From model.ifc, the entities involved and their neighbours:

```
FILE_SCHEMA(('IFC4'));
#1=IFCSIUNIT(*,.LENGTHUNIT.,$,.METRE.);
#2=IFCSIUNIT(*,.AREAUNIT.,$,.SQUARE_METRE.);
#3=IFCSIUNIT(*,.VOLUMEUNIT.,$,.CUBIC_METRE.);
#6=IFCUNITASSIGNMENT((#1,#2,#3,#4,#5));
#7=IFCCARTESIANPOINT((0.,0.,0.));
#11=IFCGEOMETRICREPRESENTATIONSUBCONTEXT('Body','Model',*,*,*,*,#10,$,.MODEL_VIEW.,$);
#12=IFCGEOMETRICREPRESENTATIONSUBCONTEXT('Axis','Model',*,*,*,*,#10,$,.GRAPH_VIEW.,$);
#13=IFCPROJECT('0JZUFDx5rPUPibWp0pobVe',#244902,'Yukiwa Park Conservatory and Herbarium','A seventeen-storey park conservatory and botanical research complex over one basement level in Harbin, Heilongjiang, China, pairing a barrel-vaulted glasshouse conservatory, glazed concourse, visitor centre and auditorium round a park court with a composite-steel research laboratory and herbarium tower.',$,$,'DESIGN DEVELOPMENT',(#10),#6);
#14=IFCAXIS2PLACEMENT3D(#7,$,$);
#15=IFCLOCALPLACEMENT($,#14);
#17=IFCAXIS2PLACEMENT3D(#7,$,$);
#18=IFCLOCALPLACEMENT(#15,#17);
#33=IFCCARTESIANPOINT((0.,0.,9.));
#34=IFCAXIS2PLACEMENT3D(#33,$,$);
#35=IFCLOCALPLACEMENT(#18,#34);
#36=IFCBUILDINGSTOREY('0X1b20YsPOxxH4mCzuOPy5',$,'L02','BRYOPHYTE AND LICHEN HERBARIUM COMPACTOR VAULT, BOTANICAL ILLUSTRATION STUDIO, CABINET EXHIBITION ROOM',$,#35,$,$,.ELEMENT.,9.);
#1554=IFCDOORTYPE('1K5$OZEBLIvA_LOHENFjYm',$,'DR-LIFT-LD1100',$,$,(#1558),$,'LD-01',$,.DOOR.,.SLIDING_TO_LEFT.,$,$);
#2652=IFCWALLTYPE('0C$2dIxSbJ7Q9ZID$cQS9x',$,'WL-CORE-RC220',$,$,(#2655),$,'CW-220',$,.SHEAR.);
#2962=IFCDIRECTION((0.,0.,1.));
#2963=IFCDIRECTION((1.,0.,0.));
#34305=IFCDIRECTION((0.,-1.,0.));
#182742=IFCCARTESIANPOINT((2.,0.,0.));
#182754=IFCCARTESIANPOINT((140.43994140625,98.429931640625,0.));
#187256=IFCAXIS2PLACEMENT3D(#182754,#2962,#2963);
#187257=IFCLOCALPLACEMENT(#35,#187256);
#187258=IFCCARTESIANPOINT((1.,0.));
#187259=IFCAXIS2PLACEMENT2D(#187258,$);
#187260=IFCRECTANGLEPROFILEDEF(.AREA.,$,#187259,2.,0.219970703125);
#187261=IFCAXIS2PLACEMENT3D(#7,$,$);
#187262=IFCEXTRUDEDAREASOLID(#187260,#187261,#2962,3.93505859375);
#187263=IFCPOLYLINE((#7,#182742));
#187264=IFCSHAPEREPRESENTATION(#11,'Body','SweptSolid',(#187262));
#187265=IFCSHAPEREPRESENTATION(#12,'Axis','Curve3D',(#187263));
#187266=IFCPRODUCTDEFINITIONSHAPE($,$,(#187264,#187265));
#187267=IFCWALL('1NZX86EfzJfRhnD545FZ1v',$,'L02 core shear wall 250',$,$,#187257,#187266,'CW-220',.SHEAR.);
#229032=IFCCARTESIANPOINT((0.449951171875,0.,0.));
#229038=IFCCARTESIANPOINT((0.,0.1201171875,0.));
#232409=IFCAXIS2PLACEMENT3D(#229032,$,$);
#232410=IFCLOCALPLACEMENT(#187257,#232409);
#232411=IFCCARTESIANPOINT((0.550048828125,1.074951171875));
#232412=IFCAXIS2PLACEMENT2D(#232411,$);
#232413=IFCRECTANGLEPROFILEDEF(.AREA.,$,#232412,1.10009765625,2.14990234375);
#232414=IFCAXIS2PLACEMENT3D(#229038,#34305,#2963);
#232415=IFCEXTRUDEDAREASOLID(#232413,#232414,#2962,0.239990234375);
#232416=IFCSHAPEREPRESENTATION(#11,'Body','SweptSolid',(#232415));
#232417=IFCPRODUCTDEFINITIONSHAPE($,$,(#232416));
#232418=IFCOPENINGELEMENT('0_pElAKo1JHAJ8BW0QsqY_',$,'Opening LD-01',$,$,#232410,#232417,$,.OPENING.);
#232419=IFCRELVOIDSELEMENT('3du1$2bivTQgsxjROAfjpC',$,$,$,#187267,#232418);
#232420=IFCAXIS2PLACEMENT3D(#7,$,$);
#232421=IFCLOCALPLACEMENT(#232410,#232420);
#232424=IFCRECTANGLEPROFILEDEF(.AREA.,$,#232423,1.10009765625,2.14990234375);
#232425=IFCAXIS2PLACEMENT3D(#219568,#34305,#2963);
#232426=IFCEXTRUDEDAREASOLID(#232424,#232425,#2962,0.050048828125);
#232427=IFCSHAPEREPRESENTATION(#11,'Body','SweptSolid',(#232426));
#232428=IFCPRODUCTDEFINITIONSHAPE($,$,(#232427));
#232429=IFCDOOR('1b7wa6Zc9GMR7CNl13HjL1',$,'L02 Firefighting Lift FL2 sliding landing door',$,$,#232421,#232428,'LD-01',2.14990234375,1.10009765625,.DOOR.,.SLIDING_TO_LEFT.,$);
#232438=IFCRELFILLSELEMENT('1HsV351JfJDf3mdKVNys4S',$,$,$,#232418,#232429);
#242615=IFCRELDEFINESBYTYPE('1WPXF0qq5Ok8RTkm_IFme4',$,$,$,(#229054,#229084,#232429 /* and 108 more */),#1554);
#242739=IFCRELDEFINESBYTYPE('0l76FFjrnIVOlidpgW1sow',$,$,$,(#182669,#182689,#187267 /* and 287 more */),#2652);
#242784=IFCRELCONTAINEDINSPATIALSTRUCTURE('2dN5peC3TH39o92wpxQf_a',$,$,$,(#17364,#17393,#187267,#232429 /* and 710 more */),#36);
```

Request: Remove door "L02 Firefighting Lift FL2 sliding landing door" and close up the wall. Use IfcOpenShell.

```python
import ifcopenshell
import ifcopenshell.api.feature
import ifcopenshell.api.root
import ifcopenshell.geom
import ifcopenshell.util.shape

model = ifcopenshell.open("model.ifc")
settings = ifcopenshell.geom.settings()


def volume(element):
    """Net volume in cubic metres, openings subtracted."""
    shape = ifcopenshell.geom.create_shape(settings, element)
    return ifcopenshell.util.shape.get_volume(shape.geometry)


door = model.by_id(232429)
opening = door.FillsVoids[0].RelatingOpeningElement
wall = opening.VoidsElements[0].RelatingBuildingElement
before = volume(wall)

ifcopenshell.api.root.remove_product(model, product=door)
ifcopenshell.api.feature.remove_feature(model, feature=opening)

after = volume(wall)

print(f"wall volume {before:.3f} -> {after:.3f} m3")

model.write("model-out.ifc")
```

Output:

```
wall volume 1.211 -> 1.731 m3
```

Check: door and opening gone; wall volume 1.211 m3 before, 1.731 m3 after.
